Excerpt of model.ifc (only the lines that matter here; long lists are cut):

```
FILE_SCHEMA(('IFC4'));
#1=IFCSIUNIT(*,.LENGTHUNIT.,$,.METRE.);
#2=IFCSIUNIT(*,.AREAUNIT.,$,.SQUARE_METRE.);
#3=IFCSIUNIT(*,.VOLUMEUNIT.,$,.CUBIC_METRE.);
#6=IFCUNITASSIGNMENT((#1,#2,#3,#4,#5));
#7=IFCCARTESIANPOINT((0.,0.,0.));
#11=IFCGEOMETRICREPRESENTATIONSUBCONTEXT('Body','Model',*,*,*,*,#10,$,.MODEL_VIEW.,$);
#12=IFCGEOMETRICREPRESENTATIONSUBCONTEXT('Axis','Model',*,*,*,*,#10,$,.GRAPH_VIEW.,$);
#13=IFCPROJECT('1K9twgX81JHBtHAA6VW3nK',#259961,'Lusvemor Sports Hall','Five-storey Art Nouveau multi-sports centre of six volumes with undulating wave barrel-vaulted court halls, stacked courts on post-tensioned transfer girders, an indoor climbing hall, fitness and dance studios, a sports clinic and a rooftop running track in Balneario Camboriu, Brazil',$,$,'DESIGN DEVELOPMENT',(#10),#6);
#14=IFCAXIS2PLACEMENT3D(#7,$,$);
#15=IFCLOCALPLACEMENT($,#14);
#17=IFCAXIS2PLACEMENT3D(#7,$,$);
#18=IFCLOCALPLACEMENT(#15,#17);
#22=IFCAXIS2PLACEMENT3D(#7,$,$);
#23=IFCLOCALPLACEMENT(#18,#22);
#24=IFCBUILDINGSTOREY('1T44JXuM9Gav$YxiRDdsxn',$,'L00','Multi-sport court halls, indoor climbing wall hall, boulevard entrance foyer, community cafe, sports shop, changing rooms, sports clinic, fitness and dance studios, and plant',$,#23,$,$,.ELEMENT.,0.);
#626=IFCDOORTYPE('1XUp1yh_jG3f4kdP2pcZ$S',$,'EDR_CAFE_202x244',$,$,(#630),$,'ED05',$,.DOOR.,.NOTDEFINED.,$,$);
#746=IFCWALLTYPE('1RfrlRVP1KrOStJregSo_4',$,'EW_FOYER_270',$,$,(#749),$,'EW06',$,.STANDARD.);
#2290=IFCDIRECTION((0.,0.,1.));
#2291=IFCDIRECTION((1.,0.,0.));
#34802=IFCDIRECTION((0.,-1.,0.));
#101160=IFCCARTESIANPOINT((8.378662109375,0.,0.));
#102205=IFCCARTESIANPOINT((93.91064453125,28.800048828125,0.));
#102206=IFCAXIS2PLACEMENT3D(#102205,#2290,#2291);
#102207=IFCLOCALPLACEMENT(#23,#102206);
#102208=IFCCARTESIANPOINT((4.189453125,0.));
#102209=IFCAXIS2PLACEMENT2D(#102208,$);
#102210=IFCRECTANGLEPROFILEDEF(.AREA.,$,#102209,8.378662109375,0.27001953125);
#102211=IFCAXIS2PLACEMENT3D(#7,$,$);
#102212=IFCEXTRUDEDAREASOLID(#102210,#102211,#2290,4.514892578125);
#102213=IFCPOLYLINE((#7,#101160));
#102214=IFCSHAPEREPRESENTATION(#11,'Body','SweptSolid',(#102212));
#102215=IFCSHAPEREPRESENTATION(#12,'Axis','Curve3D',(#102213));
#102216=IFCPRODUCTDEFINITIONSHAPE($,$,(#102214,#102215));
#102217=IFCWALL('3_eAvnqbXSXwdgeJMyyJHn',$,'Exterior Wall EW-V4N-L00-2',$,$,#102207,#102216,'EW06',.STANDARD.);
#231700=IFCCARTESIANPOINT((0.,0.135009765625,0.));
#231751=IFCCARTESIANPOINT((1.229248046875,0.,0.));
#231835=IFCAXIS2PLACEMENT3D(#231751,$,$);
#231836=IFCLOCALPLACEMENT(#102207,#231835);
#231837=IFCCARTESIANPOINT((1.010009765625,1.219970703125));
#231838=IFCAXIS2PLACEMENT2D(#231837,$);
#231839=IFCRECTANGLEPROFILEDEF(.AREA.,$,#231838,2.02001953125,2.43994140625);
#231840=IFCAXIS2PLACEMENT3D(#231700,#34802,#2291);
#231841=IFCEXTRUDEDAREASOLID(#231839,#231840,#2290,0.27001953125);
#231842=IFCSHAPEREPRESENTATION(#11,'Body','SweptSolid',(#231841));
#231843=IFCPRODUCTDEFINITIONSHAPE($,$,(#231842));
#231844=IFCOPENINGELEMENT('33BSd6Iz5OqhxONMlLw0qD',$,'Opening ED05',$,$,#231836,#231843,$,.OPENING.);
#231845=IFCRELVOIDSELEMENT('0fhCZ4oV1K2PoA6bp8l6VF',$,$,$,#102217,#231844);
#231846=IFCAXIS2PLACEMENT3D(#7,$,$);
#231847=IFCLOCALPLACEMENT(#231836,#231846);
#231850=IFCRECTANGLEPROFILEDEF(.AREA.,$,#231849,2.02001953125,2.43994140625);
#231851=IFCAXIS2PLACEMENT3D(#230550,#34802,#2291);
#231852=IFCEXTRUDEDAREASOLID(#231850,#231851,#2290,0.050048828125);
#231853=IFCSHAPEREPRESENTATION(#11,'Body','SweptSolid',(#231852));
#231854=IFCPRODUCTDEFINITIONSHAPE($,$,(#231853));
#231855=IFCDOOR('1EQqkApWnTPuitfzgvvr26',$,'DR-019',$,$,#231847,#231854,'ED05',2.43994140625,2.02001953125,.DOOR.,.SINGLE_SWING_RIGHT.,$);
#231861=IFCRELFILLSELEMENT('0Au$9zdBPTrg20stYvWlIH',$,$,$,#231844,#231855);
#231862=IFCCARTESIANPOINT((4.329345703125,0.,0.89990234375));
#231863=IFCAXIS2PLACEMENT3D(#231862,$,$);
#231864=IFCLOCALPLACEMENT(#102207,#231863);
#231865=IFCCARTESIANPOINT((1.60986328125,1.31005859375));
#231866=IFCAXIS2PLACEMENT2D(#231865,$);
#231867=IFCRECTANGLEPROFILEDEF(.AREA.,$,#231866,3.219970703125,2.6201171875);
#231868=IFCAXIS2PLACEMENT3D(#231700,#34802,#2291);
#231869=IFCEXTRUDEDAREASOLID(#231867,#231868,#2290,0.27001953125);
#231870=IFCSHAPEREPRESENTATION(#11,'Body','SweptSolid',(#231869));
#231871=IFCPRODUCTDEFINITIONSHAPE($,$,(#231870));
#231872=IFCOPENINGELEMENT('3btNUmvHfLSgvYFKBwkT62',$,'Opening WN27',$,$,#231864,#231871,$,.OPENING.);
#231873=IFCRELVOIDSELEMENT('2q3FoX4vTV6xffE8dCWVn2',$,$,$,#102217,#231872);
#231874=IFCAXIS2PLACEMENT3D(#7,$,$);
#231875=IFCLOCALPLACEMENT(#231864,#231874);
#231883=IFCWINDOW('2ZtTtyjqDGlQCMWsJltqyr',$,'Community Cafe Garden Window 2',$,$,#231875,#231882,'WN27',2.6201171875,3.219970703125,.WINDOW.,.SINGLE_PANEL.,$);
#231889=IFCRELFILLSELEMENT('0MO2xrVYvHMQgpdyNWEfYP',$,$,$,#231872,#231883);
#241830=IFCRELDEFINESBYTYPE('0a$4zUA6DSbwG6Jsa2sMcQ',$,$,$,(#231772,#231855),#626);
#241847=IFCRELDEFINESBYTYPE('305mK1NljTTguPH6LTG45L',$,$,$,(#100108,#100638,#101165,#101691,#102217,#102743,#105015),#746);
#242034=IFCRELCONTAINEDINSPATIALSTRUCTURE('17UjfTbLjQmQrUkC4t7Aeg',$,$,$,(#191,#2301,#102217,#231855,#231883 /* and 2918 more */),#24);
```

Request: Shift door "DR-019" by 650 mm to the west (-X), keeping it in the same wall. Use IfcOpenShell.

```python
import ifcopenshell
import ifcopenshell.api.geometry
import ifcopenshell.util.placement
import ifcopenshell.util.unit

model = ifcopenshell.open("model.ifc")
unit_scale = ifcopenshell.util.unit.calculate_unit_scale(model)

door = model.by_guid("1EQqkApWnTPuitfzgvvr26")
opening = door.FillsVoids[0].RelatingOpeningElement
wall = opening.VoidsElements[0].RelatingBuildingElement

wall_matrix = ifcopenshell.util.placement.get_local_placement(wall.ObjectPlacement)
shift = wall_matrix[:3, 0] * -0.65 / unit_scale
before = ifcopenshell.util.placement.get_local_placement(door.ObjectPlacement)[:3, 3].copy()

# The door is placed relative to its opening, so it follows when the opening moves.
matrix = ifcopenshell.util.placement.get_local_placement(opening.ObjectPlacement)
matrix[:3, 3] += shift
ifcopenshell.api.geometry.edit_object_placement(
    model, product=opening, matrix=matrix, is_si=False, should_transform_children=True
)

after = ifcopenshell.util.placement.get_local_placement(door.ObjectPlacement)[:3, 3]
print("door moved by", (after - before).round(3) + 0.0)

model.write("model_v2.ifc")
```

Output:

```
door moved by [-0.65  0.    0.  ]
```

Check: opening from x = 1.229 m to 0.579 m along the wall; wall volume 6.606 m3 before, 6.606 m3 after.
